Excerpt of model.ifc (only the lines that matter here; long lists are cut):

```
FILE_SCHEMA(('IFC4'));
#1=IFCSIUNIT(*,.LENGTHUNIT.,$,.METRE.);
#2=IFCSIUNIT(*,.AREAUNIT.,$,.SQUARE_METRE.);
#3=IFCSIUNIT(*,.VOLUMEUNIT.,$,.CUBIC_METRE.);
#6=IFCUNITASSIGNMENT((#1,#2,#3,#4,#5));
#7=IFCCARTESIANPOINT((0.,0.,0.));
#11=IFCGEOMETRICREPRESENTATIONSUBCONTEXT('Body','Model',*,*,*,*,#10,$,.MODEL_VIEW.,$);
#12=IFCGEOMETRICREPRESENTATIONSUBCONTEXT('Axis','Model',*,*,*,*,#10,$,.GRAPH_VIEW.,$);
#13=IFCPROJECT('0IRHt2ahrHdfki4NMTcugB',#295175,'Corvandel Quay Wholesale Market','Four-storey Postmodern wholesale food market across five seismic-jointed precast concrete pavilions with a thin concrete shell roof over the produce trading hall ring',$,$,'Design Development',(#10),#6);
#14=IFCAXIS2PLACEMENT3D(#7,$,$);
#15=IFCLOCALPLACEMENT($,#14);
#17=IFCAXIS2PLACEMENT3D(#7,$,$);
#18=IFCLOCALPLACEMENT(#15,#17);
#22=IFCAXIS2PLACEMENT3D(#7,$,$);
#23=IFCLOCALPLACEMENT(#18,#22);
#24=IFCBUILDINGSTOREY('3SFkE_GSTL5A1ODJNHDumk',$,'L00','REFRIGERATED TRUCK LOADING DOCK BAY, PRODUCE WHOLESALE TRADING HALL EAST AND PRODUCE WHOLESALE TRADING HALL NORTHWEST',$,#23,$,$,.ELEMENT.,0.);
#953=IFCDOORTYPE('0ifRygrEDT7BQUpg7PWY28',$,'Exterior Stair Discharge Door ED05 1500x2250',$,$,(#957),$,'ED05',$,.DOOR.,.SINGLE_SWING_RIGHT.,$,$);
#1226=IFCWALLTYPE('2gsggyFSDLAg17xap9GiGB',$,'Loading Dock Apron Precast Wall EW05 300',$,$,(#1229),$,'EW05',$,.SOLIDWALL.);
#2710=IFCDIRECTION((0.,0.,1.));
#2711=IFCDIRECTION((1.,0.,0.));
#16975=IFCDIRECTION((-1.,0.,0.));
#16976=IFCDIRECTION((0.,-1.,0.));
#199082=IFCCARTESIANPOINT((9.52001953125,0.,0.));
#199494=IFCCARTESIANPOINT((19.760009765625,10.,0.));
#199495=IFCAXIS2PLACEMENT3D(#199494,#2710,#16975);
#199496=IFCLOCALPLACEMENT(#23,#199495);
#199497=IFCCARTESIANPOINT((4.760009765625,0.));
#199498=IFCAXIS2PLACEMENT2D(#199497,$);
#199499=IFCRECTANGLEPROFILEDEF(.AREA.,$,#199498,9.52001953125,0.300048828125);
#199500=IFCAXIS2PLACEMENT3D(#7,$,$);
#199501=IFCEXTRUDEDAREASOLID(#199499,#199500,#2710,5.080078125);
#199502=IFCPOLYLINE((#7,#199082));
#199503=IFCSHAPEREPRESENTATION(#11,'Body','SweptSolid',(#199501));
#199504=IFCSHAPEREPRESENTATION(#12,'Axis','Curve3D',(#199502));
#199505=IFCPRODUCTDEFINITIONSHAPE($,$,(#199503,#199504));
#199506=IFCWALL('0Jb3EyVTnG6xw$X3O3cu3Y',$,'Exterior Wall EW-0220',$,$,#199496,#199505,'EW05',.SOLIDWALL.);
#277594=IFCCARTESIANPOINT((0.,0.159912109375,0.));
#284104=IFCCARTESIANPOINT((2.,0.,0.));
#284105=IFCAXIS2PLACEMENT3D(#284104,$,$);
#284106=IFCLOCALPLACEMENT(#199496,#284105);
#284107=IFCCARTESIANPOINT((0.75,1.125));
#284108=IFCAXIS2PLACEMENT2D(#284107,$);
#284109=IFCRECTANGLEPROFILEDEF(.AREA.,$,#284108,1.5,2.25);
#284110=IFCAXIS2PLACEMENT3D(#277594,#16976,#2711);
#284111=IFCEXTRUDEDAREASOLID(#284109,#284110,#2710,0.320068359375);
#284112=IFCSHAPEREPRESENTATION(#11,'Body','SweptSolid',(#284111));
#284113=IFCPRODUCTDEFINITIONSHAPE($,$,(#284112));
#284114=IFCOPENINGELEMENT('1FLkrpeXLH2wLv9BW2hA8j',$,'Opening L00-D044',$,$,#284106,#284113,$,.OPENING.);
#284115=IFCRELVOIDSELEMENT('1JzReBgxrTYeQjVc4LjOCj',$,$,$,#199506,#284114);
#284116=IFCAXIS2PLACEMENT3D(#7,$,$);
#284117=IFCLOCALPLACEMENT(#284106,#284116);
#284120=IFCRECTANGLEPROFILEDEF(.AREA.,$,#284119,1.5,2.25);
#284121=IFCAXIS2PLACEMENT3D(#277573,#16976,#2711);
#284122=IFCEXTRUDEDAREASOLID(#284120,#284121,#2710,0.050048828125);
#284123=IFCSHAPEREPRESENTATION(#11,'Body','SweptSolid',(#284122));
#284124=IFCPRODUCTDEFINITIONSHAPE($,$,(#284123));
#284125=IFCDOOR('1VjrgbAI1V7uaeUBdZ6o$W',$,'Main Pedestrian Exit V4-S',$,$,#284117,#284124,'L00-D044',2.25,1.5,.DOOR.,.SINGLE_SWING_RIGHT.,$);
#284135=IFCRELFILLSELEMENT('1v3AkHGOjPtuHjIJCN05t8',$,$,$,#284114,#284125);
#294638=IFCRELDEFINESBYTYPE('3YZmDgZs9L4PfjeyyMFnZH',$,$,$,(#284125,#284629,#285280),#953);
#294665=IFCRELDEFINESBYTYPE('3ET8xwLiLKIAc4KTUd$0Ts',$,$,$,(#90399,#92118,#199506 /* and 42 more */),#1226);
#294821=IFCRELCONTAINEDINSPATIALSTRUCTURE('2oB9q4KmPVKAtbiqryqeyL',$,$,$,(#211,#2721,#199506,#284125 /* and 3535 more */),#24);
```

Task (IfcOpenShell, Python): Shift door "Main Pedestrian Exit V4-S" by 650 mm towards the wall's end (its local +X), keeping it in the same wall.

```python
import ifcopenshell
import ifcopenshell.api.geometry
import ifcopenshell.util.placement

model = ifcopenshell.open("model.ifc")

door = model.by_id(284125)
opening = door.FillsVoids[0].RelatingOpeningElement
wall = opening.VoidsElements[0].RelatingBuildingElement

wall_matrix = ifcopenshell.util.placement.get_local_placement(wall.ObjectPlacement)
shift = wall_matrix[:3, 0] * 0.65
before = ifcopenshell.util.placement.get_local_placement(door.ObjectPlacement)[:3, 3].copy()

# The door is placed relative to its opening, so it follows when the opening moves.
matrix = ifcopenshell.util.placement.get_local_placement(opening.ObjectPlacement)
matrix[:3, 3] += shift
ifcopenshell.api.geometry.edit_object_placement(
    model, product=opening, matrix=matrix, is_si=False, should_transform_children=True
)

after = ifcopenshell.util.placement.get_local_placement(door.ObjectPlacement)[:3, 3]
print("door moved by", (after - before).round(3) + 0.0)

model.write("model_edited.ifc")
```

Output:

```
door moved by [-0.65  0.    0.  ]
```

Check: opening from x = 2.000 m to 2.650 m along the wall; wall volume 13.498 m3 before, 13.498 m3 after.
